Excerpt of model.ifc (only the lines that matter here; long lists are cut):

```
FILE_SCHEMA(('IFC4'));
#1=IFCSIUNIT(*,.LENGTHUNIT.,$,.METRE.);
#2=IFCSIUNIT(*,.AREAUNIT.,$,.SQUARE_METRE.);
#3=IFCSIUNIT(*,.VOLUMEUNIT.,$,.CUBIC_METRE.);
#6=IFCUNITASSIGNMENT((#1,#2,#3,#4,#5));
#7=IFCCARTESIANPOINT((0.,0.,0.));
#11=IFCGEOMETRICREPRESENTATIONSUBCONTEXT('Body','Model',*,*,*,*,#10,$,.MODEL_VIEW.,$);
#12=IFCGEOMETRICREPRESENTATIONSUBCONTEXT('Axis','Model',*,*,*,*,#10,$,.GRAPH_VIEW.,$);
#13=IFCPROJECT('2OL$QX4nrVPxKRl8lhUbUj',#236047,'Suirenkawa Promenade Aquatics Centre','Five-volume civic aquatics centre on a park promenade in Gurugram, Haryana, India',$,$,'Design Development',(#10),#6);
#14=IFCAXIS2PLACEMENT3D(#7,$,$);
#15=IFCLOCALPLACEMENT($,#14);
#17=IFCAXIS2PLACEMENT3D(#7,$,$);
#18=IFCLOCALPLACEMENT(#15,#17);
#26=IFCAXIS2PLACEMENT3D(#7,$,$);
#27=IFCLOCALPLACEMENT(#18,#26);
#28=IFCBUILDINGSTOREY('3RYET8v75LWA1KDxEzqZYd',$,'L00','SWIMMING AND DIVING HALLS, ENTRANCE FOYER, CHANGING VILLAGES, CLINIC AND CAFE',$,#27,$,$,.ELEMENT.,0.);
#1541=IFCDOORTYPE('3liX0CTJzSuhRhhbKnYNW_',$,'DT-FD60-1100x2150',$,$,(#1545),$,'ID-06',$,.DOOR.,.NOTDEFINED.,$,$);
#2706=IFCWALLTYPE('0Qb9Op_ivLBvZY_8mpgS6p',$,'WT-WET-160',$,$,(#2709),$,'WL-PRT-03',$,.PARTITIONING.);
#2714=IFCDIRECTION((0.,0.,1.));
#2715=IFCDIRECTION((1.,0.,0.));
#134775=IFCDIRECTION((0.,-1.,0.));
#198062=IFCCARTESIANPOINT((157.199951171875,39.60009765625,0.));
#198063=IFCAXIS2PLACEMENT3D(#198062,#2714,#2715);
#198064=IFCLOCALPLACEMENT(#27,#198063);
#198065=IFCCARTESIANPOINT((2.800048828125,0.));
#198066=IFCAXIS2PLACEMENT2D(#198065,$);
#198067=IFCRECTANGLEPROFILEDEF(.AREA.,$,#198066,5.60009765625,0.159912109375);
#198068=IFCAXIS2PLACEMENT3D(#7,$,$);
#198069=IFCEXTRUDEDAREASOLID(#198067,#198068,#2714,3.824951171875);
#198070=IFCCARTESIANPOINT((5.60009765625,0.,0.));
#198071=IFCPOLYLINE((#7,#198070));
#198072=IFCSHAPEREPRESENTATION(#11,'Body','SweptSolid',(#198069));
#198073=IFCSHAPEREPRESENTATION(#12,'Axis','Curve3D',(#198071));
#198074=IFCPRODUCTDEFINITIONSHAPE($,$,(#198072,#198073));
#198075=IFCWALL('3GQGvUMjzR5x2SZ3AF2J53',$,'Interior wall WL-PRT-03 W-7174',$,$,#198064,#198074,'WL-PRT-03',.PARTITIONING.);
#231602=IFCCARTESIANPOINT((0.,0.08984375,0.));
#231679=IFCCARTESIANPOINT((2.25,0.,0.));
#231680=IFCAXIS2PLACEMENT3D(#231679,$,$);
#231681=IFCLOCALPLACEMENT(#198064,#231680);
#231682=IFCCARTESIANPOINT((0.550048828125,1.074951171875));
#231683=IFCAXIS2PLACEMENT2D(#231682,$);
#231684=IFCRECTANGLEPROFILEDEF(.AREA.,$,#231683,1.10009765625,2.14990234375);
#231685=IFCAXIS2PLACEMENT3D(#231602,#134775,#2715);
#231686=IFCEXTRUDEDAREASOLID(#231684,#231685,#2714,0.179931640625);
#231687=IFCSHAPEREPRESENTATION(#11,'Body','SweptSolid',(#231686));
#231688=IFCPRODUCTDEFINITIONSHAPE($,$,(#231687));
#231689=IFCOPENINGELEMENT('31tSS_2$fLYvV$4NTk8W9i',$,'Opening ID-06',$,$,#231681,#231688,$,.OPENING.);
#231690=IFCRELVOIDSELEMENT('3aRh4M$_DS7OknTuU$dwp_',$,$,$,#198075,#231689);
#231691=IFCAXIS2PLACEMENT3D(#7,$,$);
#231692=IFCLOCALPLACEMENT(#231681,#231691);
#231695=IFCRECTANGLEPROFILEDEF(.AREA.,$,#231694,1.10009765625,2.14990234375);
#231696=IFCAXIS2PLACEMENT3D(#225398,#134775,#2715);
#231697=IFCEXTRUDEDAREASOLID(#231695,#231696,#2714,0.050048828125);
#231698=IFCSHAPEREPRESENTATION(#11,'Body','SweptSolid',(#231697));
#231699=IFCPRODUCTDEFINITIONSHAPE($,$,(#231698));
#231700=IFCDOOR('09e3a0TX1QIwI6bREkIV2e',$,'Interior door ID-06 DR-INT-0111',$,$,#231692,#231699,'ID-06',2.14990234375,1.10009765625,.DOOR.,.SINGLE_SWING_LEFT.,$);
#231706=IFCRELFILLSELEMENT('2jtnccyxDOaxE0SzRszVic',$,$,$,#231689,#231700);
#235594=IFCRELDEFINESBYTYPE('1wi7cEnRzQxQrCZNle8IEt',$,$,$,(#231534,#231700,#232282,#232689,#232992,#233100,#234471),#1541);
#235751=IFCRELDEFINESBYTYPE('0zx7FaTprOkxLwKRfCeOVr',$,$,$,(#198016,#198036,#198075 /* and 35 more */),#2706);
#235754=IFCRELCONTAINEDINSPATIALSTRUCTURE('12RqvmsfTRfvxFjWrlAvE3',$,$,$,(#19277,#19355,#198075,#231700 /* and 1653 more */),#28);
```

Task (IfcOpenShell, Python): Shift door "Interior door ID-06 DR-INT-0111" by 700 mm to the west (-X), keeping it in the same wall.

```python
import ifcopenshell
import ifcopenshell.api.geometry
import ifcopenshell.util.placement

model = ifcopenshell.open("model.ifc")

door = model.by_id(231700)
opening = door.FillsVoids[0].RelatingOpeningElement
wall = opening.VoidsElements[0].RelatingBuildingElement

wall_matrix = ifcopenshell.util.placement.get_local_placement(wall.ObjectPlacement)
shift = wall_matrix[:3, 0] * -0.7
before = ifcopenshell.util.placement.get_local_placement(door.ObjectPlacement)[:3, 3].copy()

# The door is placed relative to its opening, so it follows when the opening moves.
matrix = ifcopenshell.util.placement.get_local_placement(opening.ObjectPlacement)
matrix[:3, 3] += shift
ifcopenshell.api.geometry.edit_object_placement(
    model, product=opening, matrix=matrix, is_si=False, should_transform_children=True
)

after = ifcopenshell.util.placement.get_local_placement(door.ObjectPlacement)[:3, 3]
print("door moved by", (after - before).round(3) + 0.0)

model.write("model_edited.ifc")
```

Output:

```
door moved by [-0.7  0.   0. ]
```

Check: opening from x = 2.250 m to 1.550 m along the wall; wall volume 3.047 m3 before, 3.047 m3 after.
